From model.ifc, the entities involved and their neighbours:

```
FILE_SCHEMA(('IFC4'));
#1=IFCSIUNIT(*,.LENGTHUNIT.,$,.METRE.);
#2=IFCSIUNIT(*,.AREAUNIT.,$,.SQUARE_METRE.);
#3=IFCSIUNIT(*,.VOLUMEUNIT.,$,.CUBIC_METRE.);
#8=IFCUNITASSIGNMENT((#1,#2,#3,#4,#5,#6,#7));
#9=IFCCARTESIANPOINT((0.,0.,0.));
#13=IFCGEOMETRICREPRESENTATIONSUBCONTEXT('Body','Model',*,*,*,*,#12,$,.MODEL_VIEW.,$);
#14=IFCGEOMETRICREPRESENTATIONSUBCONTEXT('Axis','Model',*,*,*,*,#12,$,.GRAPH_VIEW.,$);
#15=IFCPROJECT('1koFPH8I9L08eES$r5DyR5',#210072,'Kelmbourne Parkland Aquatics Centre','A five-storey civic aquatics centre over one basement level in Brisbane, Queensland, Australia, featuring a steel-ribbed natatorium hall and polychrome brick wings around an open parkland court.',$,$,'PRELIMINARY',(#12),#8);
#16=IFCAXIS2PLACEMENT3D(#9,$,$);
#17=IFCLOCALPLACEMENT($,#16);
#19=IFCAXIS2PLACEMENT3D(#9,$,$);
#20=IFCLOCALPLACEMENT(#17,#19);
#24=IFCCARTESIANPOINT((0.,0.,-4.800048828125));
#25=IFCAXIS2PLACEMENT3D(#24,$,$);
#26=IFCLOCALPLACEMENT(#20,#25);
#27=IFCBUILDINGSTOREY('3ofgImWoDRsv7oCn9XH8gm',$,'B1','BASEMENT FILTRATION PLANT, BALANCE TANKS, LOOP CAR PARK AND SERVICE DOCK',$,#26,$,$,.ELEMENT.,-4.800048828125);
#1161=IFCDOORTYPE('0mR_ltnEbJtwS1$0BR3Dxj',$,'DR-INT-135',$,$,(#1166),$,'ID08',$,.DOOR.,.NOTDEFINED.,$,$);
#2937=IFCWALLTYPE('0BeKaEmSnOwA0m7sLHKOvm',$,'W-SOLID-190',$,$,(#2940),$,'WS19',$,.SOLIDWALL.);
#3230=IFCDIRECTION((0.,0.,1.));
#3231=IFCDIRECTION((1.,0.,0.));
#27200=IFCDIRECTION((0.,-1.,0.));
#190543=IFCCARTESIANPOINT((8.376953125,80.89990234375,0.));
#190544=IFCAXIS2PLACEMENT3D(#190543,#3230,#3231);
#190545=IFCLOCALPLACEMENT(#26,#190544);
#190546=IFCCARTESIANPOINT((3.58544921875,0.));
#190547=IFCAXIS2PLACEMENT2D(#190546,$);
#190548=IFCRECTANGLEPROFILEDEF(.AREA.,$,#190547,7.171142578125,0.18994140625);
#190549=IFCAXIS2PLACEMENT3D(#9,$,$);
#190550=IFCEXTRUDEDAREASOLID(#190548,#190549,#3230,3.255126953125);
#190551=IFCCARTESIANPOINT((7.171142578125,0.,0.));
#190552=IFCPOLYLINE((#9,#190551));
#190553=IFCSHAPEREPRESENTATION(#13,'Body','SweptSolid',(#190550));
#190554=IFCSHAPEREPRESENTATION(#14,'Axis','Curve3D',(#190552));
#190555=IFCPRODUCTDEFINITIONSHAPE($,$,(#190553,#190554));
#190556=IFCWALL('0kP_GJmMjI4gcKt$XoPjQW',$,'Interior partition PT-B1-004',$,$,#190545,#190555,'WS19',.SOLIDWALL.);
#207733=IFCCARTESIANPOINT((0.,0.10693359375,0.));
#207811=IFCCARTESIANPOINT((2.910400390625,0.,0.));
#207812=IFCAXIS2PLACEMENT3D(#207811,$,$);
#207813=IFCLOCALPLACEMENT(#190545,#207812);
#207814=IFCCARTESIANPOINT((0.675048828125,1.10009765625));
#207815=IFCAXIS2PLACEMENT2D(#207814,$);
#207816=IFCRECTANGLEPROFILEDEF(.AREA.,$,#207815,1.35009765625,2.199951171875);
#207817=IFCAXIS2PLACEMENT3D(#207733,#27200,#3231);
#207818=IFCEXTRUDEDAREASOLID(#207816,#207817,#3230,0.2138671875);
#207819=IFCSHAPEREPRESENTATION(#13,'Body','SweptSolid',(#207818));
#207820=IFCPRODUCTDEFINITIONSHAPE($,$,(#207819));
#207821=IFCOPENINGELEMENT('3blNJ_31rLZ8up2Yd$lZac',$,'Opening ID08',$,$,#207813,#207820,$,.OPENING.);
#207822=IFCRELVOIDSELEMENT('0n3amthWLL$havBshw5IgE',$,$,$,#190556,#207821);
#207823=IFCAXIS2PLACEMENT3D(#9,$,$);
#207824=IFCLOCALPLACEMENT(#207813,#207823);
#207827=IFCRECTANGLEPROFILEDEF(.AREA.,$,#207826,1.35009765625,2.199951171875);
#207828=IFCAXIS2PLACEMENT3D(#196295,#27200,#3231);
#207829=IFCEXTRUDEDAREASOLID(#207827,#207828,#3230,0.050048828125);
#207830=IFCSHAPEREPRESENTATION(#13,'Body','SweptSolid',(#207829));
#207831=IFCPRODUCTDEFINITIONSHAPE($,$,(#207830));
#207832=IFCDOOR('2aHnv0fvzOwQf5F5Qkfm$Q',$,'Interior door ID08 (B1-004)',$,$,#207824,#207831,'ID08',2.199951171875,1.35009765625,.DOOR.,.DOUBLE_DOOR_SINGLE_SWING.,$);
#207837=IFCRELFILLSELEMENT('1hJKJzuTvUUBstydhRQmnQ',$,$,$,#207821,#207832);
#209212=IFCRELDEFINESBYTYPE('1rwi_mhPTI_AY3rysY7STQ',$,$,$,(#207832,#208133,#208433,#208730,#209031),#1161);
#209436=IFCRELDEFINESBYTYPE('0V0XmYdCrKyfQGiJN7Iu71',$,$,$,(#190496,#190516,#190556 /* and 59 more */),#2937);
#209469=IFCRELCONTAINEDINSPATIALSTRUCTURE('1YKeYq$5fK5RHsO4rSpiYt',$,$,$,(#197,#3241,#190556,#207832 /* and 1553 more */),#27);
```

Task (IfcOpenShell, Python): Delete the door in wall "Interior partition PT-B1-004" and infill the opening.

```python
import ifcopenshell
import ifcopenshell.api.feature
import ifcopenshell.api.root
import ifcopenshell.geom
import ifcopenshell.util.shape

model = ifcopenshell.open("model.ifc")
settings = ifcopenshell.geom.settings()


def volume(element):
    """Net volume in cubic metres, openings subtracted."""
    shape = ifcopenshell.geom.create_shape(settings, element)
    return ifcopenshell.util.shape.get_volume(shape.geometry)


door = model.by_guid("2aHnv0fvzOwQf5F5Qkfm$Q")
opening = door.FillsVoids[0].RelatingOpeningElement
wall = opening.VoidsElements[0].RelatingBuildingElement
before = volume(wall)

ifcopenshell.api.root.remove_product(model, product=door)
ifcopenshell.api.feature.remove_feature(model, feature=opening)

after = volume(wall)

print(f"wall volume {before:.3f} -> {after:.3f} m3")

model.write("model_rev.ifc")
```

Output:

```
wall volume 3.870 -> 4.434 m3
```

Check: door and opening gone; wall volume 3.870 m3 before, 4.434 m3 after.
